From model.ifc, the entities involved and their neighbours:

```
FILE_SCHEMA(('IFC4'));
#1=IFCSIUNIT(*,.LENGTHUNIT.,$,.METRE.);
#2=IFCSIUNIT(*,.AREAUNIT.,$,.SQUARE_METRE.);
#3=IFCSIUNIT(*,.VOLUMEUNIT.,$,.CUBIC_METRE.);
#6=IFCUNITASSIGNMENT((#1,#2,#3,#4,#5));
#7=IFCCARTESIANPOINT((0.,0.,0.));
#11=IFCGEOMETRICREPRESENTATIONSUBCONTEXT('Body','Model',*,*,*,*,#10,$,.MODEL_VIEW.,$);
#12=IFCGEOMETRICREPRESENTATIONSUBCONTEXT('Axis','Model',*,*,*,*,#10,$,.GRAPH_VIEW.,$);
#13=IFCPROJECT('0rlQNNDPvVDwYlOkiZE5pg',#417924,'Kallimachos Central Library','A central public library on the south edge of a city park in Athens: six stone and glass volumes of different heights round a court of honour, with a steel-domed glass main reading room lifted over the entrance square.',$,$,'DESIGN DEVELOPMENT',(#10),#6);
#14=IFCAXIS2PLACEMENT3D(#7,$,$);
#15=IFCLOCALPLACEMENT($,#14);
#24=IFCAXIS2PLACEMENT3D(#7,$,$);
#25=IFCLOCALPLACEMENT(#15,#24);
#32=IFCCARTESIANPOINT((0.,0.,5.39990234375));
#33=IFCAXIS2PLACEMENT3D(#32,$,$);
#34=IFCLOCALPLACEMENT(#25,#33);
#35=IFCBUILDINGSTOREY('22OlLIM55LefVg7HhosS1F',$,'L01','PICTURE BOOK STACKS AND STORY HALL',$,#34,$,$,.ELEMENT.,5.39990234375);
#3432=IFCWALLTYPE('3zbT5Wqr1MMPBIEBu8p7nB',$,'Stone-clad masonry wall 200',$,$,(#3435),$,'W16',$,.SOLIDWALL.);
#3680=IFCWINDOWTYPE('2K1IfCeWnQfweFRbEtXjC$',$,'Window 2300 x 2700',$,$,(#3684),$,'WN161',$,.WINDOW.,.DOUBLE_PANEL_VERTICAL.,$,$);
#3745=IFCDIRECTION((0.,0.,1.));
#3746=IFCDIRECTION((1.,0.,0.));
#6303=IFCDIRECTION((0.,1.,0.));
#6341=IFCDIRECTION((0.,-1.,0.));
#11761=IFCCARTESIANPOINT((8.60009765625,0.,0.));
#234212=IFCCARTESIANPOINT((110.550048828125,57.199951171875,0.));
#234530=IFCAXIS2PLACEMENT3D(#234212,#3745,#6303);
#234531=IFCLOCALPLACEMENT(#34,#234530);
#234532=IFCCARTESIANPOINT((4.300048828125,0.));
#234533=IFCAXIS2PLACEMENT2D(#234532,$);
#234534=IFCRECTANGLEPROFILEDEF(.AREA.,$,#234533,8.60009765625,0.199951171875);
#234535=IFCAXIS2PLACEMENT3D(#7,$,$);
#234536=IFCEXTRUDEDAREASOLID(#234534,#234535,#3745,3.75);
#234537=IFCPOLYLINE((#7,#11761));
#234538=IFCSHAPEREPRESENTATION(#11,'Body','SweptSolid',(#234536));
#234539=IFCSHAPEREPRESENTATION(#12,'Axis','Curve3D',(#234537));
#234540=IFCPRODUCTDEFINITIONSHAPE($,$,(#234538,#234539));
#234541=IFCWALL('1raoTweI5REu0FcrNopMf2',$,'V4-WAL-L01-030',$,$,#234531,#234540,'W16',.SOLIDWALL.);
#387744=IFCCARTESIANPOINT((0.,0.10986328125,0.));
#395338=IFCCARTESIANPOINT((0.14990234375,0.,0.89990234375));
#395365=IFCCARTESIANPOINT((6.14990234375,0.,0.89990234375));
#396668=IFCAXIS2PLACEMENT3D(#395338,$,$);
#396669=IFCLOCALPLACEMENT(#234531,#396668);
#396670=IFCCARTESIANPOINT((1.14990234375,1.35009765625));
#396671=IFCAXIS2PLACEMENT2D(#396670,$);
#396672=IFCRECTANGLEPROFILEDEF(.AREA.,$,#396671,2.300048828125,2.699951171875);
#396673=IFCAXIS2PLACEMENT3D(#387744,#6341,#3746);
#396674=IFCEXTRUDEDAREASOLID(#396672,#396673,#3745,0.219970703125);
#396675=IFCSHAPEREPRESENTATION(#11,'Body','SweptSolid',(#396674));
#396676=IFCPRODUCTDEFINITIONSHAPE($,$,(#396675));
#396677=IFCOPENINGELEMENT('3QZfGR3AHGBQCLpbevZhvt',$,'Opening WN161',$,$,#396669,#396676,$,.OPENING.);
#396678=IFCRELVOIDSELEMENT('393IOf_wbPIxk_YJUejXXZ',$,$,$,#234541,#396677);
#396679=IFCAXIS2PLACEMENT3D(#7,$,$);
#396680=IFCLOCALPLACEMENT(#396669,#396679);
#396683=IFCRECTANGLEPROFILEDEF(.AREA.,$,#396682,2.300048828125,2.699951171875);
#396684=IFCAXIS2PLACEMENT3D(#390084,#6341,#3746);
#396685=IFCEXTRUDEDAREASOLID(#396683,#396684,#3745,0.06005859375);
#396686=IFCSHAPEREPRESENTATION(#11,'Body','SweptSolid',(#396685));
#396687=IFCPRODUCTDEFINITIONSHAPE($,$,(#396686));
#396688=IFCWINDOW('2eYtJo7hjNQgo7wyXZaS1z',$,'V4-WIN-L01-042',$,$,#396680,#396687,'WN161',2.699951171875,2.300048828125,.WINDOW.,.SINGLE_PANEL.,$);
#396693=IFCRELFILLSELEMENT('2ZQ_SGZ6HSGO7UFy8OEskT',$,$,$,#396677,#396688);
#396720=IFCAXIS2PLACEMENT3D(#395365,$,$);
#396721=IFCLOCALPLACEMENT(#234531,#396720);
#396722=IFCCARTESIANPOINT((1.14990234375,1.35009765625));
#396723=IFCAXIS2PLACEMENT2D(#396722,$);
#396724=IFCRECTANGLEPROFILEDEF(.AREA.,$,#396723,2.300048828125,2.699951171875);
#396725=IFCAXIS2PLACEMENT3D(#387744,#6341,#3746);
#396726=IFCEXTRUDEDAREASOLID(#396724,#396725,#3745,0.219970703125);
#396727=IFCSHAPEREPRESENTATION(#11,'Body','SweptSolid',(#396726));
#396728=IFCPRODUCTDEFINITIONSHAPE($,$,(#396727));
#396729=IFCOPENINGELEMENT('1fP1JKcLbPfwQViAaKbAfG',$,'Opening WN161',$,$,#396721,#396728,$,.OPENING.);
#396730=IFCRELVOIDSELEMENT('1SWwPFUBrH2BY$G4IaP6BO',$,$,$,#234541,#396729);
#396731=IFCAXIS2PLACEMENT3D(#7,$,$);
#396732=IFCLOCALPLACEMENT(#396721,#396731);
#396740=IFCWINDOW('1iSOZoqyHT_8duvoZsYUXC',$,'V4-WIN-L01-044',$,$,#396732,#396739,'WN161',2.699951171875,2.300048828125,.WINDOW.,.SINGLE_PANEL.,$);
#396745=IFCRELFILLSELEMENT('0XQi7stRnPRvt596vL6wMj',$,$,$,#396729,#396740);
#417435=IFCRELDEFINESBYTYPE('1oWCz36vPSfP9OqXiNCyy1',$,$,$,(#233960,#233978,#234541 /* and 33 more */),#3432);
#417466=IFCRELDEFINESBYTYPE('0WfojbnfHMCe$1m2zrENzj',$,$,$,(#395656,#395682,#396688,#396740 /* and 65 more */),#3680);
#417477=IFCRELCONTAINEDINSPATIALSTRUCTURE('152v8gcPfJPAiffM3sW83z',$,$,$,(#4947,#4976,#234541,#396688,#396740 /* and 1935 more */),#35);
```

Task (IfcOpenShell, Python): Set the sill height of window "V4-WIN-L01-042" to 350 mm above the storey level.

```python
import numpy as np
import ifcopenshell
import ifcopenshell.api.geometry
import ifcopenshell.geom
import ifcopenshell.util.element
import ifcopenshell.util.placement
import ifcopenshell.util.shape
import ifcopenshell.util.unit

model = ifcopenshell.open("model.ifc")
unit_scale = ifcopenshell.util.unit.calculate_unit_scale(model)

window = model.by_guid("2eYtJo7hjNQgo7wyXZaS1z")
opening = window.FillsVoids[0].RelatingOpeningElement
storey = ifcopenshell.util.element.get_container(window, ifc_class="IfcBuildingStorey")
level = ifcopenshell.util.placement.get_local_placement(storey.ObjectPlacement)[2, 3]

# The opening's origin need not be at the sill, so measure its lowest point.
shape = ifcopenshell.geom.create_shape(ifcopenshell.geom.settings(), opening)
bottom = ifcopenshell.util.shape.get_shape_bottom_elevation(shape, shape.geometry) / unit_scale
dz = level + 0.35 / unit_scale - bottom

shift = np.array([0.0, 0.0, dz])
# The window is placed relative to its opening, so it follows when the opening moves.
matrix = ifcopenshell.util.placement.get_local_placement(opening.ObjectPlacement)
matrix[:3, 3] += shift
ifcopenshell.api.geometry.edit_object_placement(
    model, product=opening, matrix=matrix, is_si=False, should_transform_children=True
)

print(f"moved by {dz * unit_scale:+.3f} m")

model.write("model_v2.ifc")
```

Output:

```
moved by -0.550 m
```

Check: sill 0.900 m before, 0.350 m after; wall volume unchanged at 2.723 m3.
